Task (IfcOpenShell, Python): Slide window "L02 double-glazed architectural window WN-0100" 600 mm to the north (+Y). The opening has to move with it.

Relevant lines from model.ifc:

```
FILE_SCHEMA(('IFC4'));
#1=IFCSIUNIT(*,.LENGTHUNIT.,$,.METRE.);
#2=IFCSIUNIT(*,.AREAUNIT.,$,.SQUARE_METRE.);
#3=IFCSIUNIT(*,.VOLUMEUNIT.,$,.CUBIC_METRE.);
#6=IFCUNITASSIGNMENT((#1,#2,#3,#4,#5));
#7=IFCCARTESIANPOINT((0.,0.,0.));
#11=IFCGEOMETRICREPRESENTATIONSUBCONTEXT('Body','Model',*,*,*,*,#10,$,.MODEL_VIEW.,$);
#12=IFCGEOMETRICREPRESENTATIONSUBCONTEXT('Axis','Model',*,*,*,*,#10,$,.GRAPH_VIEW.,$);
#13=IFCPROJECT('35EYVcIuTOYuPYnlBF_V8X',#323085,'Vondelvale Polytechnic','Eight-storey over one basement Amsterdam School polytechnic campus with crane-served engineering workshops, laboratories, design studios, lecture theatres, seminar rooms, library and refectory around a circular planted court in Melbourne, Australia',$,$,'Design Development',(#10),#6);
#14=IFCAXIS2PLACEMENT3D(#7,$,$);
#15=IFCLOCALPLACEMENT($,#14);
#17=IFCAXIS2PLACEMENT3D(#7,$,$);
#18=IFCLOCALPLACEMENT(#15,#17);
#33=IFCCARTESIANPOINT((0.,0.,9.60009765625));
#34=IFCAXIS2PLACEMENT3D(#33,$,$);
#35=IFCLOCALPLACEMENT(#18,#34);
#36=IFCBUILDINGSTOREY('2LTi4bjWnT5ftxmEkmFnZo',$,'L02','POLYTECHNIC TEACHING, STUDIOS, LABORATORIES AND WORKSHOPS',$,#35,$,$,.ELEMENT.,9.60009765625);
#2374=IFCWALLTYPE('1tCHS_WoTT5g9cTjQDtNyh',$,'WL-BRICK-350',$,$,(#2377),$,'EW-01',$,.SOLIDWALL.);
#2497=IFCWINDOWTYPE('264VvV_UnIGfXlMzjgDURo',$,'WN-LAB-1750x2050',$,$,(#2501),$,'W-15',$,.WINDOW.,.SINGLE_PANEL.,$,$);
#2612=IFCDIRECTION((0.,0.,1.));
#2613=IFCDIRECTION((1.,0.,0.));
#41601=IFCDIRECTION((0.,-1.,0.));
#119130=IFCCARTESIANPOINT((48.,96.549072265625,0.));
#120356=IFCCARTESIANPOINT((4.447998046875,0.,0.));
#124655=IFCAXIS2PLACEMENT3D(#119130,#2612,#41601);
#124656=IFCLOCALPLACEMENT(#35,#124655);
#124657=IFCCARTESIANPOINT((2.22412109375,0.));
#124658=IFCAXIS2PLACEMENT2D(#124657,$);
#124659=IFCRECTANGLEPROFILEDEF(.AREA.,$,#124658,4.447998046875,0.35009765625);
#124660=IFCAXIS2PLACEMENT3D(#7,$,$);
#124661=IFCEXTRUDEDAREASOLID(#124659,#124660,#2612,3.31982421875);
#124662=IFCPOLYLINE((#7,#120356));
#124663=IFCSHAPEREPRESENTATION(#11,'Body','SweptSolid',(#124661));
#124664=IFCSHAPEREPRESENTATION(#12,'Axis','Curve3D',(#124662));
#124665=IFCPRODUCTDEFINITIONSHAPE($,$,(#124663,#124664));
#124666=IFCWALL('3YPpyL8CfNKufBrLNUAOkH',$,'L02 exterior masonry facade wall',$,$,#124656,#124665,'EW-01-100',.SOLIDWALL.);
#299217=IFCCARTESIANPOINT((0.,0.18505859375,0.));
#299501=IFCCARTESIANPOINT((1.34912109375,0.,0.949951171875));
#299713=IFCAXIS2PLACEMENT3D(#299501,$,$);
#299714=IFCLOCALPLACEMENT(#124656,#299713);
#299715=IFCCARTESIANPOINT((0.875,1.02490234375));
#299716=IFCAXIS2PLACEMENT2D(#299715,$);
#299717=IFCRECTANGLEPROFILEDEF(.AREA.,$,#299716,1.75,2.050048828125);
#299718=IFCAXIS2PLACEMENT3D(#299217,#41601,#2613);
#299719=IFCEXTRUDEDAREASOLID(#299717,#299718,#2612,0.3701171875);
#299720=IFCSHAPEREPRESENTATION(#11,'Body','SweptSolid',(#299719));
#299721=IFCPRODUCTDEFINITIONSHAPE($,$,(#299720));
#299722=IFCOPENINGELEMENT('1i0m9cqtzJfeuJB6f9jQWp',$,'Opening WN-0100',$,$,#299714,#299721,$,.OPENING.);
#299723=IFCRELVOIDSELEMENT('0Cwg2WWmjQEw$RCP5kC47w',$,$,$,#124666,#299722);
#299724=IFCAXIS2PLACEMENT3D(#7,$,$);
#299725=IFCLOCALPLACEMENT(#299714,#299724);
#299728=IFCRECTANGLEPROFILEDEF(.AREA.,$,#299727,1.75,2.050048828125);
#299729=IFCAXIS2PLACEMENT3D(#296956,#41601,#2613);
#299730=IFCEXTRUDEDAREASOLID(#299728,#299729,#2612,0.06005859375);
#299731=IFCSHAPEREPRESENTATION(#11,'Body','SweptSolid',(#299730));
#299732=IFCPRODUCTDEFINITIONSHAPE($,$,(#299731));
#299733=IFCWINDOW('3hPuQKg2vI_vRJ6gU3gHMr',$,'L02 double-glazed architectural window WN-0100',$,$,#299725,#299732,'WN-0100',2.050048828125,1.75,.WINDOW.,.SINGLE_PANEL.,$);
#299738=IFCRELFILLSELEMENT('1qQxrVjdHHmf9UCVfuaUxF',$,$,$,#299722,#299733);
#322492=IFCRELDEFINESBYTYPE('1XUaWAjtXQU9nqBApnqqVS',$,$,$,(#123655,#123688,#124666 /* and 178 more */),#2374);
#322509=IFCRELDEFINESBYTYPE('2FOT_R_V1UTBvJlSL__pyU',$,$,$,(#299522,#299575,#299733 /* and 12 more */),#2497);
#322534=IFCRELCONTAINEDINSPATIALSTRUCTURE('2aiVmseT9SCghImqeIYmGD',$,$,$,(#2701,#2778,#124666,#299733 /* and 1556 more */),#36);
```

```python
import ifcopenshell
import ifcopenshell.api.geometry
import ifcopenshell.util.placement

model = ifcopenshell.open("model.ifc")

window = model.by_guid("3hPuQKg2vI_vRJ6gU3gHMr")
opening = window.FillsVoids[0].RelatingOpeningElement
wall = opening.VoidsElements[0].RelatingBuildingElement

wall_matrix = ifcopenshell.util.placement.get_local_placement(wall.ObjectPlacement)
shift = wall_matrix[:3, 0] * -0.6
before = ifcopenshell.util.placement.get_local_placement(window.ObjectPlacement)[:3, 3].copy()

# The window is placed relative to its opening, so it follows when the opening moves.
matrix = ifcopenshell.util.placement.get_local_placement(opening.ObjectPlacement)
matrix[:3, 3] += shift
ifcopenshell.api.geometry.edit_object_placement(
    model, product=opening, matrix=matrix, is_si=False, should_transform_children=True
)

after = ifcopenshell.util.placement.get_local_placement(window.ObjectPlacement)[:3, 3]
print("window moved by", (after - before).round(3) + 0.0)

model.write("model_v2.ifc")
```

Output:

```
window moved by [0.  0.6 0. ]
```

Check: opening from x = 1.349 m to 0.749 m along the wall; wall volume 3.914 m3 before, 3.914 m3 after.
